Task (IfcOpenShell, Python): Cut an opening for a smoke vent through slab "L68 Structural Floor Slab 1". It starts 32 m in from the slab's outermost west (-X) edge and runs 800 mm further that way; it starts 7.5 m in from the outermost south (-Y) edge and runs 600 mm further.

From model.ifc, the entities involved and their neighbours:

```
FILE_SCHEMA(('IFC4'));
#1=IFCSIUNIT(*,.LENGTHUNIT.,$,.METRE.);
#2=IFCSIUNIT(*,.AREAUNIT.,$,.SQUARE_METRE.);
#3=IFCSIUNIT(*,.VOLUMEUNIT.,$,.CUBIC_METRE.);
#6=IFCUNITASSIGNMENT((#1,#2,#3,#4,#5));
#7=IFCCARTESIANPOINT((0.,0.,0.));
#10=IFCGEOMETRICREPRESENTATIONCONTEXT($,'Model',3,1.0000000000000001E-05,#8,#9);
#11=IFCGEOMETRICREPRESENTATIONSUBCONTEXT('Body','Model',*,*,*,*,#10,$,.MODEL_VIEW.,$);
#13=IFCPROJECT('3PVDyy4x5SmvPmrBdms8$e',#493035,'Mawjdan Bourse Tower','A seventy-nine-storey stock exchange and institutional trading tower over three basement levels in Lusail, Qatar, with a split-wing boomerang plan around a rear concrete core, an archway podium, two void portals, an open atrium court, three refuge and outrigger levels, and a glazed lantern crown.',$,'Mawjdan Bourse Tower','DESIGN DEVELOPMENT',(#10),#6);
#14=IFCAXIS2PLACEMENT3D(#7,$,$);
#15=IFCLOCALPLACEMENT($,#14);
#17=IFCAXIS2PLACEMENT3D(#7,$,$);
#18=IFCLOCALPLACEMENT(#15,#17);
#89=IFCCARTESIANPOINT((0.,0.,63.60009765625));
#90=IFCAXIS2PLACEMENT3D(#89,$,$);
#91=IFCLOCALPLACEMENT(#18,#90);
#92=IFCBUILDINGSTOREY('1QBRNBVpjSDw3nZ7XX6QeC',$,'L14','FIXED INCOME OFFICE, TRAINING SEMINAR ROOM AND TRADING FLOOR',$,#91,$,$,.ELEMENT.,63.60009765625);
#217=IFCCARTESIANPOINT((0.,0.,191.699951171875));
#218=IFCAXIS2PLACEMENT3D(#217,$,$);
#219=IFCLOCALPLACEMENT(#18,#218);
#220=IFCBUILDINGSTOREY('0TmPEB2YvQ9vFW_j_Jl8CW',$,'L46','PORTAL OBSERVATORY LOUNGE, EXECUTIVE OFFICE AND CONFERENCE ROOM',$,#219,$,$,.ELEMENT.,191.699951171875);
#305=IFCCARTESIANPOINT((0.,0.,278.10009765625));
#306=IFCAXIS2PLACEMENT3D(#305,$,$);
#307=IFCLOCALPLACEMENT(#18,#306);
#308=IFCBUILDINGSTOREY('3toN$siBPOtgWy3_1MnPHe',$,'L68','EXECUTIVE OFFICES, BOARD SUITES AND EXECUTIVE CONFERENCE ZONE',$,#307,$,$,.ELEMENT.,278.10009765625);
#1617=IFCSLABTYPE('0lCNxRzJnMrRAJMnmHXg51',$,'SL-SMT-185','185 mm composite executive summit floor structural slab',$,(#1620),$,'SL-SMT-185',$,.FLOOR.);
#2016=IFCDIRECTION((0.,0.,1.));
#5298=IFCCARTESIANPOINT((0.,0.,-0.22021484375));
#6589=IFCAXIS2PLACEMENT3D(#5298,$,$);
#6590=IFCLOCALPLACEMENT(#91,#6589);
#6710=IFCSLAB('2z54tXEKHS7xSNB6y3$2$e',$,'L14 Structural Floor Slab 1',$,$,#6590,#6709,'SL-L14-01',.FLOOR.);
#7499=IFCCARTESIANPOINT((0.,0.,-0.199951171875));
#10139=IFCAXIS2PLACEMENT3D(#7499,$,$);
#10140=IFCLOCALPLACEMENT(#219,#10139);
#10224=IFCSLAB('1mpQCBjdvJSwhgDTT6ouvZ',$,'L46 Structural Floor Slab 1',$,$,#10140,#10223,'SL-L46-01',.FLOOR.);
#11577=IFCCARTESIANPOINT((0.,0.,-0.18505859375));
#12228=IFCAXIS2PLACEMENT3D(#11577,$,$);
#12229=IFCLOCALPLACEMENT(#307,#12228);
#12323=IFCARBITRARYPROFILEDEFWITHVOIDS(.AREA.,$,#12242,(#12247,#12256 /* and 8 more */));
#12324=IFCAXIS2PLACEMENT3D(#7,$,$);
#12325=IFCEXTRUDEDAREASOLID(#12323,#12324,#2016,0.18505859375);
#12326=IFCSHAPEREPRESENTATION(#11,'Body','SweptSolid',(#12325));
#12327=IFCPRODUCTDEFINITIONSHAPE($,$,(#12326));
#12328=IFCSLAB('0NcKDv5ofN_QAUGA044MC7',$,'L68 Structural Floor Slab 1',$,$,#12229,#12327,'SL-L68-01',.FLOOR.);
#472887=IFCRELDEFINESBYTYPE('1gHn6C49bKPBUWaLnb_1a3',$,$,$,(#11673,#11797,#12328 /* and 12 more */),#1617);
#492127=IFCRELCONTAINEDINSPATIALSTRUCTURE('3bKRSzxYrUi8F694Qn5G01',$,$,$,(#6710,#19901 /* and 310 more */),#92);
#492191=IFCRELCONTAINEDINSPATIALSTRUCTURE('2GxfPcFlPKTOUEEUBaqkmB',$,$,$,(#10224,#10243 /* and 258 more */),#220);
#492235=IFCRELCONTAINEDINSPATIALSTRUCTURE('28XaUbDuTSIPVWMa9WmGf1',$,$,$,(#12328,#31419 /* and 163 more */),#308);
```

```python
import numpy as np
import ifcopenshell
import ifcopenshell.api.feature
import ifcopenshell.api.geometry
import ifcopenshell.api.root
import ifcopenshell.geom
import ifcopenshell.util.placement
import ifcopenshell.util.representation
import ifcopenshell.util.shape
import ifcopenshell.util.unit

model = ifcopenshell.open("model.ifc")
unit_scale = ifcopenshell.util.unit.calculate_unit_scale(model)
settings = ifcopenshell.geom.settings()


def volume(element):
    """Net volume in cubic metres, openings subtracted."""
    shape = ifcopenshell.geom.create_shape(settings, element)
    return ifcopenshell.util.shape.get_volume(shape.geometry)


slab = model.by_id(12328)
before = volume(slab)

# Extent in the slab's own axes, in metres. The edges named are its -X and -Y sides.
slab_shape = ifcopenshell.geom.create_shape(settings, slab)
vertices = ifcopenshell.util.shape.get_vertices(slab_shape.geometry)
x_min, y_min, bottom = vertices.min(axis=0)
top = vertices[:, 2].max()

opening = ifcopenshell.api.root.create_entity(model, ifc_class="IfcOpeningElement", name="Smoke vent opening", predefined_type="OPENING")
context = ifcopenshell.util.representation.get_context(model, "Model", "Body", "MODEL_VIEW")
width, depth = 0.8, 0.6
outline = [(0.0, 0.0), (width, 0.0), (width, depth), (0.0, depth), (0.0, 0.0)]
# Overshoot both faces by 50 mm so the cut is clean.
shape = ifcopenshell.api.geometry.add_slab_representation(
    model, context=context, depth=top - bottom + 0.1, polyline=outline
)
ifcopenshell.api.geometry.assign_representation(model, product=opening, representation=shape)

matrix = ifcopenshell.util.placement.get_local_placement(slab.ObjectPlacement)
matrix[:, 3] = matrix @ np.append(np.array([x_min + 32, y_min + 7.5, bottom - 0.05]) / unit_scale, 1.0)
ifcopenshell.api.geometry.edit_object_placement(model, product=opening, matrix=matrix, is_si=False)
ifcopenshell.api.feature.add_feature(model, feature=opening, element=slab)

after = volume(slab)

print(f"slab volume {before:.3f} -> {after:.3f} m3")

model.write("model-out.ifc")
```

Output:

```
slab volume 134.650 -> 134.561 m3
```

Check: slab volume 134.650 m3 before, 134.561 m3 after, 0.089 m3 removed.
